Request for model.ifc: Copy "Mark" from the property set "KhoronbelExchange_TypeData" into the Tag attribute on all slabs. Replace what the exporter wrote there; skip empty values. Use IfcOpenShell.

First a look at what the model holds.

```python
import ifcopenshell
import ifcopenshell.util.element

model = ifcopenshell.open("model.ifc")
print(model.schema)
slabs = model.by_type("IfcSlab")
print(len(slabs), "slabs")
for e in slabs[:8]:
    source = ifcopenshell.util.element.get_pset(e, "KhoronbelExchange_TypeData", "Mark")
    target = e.Tag
    print(e.id(), repr(source), repr(target), sep=" | ")
```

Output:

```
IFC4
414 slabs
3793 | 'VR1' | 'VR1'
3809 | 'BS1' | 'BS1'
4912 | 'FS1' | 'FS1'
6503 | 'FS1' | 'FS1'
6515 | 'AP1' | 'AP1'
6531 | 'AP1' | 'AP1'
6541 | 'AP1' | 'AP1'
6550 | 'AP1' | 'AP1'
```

```python
import ifcopenshell
import ifcopenshell.util.element

model = ifcopenshell.open("model.ifc")

count = 0
for e in model.by_type("IfcSlab"):
    value = ifcopenshell.util.element.get_pset(e, "KhoronbelExchange_TypeData", "Mark")
    current = e.Tag
    if not value or not value.strip() or current == value:
        continue
    e.Tag = value
    count += 1

print(count, "slabs updated")

model.write("model_v2.ifc")
```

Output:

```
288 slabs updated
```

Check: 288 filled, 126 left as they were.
